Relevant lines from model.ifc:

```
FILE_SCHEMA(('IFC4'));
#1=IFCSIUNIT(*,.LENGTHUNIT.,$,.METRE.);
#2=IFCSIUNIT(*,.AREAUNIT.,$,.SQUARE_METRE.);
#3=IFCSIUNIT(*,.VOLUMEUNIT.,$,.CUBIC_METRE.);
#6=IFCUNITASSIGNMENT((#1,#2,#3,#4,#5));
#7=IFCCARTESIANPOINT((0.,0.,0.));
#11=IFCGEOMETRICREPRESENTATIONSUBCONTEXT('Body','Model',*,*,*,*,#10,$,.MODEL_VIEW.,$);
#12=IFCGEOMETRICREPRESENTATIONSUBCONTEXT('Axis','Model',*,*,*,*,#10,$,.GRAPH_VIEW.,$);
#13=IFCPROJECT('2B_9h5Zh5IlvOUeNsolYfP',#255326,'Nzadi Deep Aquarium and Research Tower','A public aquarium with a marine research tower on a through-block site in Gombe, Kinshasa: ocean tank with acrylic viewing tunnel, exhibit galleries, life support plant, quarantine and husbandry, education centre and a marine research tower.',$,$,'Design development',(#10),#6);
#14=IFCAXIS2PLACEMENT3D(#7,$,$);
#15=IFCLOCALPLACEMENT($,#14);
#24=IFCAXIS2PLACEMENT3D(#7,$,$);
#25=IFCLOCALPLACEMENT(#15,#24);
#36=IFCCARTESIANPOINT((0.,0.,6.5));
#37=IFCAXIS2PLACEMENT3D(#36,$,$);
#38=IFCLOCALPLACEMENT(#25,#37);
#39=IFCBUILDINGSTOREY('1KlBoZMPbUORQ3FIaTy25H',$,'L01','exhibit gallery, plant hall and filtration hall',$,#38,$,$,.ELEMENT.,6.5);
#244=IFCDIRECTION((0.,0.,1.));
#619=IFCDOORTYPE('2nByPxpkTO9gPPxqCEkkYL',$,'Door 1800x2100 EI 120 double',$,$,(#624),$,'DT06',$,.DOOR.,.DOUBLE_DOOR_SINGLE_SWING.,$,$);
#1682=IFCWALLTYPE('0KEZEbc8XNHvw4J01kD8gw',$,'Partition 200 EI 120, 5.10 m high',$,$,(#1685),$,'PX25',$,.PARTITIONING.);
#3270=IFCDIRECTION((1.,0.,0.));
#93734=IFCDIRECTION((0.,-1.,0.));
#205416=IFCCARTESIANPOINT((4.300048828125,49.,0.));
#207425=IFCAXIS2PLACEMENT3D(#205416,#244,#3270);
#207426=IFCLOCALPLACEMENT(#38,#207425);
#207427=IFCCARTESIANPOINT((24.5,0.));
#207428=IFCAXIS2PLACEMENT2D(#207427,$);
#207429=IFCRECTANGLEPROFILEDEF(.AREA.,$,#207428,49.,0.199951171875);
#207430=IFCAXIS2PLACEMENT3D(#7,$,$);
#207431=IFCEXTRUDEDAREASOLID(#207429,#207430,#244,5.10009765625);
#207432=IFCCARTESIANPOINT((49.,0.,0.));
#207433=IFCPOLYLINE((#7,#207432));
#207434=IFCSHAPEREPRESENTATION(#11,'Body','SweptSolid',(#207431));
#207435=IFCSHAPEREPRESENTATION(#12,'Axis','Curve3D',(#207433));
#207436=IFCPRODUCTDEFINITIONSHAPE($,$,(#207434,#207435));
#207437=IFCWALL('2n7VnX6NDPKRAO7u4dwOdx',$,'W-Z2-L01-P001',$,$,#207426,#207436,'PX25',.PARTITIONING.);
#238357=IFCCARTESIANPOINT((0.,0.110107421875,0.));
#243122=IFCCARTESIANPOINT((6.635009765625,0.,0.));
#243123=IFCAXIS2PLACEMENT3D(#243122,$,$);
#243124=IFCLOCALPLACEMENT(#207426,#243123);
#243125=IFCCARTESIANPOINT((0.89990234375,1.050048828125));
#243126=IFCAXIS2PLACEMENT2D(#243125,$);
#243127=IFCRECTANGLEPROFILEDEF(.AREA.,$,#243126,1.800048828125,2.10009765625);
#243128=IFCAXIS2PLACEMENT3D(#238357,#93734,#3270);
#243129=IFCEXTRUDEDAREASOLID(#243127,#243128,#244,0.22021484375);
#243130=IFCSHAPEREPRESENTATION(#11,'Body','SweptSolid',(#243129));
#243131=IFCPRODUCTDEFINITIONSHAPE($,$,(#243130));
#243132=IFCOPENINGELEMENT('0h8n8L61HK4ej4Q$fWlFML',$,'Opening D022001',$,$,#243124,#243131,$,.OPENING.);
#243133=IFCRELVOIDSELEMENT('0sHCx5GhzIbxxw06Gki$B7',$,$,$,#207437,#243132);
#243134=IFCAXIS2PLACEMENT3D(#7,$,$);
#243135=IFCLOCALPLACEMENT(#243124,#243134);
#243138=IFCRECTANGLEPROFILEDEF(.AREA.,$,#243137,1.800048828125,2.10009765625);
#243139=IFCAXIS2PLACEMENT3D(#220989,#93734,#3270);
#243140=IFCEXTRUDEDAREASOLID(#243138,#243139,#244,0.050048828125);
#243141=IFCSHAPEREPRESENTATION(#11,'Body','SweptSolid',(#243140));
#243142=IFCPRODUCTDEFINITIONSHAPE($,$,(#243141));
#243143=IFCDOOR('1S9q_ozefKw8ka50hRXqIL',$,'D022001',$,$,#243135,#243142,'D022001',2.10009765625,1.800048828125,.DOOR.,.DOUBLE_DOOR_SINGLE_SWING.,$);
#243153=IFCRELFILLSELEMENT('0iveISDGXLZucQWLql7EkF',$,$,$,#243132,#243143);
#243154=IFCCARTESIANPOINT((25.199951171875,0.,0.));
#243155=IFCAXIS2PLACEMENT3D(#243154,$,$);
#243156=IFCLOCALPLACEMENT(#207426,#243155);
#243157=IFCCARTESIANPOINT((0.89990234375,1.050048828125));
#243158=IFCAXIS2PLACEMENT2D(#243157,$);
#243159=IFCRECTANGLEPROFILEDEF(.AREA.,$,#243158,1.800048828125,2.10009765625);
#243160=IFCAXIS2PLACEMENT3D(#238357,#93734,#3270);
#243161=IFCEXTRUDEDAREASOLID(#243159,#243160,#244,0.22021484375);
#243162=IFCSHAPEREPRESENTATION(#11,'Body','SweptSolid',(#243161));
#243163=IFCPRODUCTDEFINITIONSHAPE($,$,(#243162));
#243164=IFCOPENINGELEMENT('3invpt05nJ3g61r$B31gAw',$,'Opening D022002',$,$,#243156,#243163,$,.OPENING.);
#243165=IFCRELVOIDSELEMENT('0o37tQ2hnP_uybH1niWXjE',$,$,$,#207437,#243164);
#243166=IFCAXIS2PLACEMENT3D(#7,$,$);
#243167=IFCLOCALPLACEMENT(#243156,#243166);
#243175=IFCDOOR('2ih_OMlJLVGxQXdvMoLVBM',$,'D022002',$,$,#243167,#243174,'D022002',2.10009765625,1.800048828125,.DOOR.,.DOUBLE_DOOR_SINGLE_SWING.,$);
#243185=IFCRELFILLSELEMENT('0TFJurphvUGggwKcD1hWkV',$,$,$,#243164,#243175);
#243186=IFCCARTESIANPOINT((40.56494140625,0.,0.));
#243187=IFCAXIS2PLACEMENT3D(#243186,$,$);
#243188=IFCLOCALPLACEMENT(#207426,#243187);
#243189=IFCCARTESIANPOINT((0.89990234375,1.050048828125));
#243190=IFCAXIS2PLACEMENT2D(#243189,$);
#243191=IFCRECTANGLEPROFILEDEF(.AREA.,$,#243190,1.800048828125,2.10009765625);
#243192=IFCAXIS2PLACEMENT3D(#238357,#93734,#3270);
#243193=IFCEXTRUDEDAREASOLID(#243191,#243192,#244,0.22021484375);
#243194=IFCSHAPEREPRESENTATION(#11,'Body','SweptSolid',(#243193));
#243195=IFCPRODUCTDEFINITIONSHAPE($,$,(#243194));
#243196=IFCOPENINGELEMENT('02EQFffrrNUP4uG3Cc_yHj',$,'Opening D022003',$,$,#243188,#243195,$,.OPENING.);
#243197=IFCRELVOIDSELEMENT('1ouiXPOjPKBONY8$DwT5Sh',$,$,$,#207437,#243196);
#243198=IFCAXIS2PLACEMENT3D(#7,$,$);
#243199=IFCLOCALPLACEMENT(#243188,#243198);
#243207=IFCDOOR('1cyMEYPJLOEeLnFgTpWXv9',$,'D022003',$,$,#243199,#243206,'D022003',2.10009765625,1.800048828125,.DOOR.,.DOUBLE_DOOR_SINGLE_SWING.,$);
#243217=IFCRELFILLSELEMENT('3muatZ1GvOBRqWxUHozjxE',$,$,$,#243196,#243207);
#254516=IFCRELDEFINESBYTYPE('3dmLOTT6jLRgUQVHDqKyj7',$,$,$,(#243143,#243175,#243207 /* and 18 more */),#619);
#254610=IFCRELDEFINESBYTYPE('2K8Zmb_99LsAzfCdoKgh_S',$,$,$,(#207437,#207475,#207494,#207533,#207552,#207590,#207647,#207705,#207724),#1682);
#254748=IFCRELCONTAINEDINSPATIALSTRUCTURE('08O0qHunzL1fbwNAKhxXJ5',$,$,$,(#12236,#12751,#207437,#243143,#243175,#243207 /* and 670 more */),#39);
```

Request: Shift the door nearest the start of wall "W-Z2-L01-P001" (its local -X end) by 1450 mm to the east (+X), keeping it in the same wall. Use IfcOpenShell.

```python
import ifcopenshell
import ifcopenshell.api.geometry
import ifcopenshell.util.placement

model = ifcopenshell.open("model.ifc")

door = model.by_guid("1S9q_ozefKw8ka50hRXqIL")
opening = door.FillsVoids[0].RelatingOpeningElement
wall = opening.VoidsElements[0].RelatingBuildingElement

wall_matrix = ifcopenshell.util.placement.get_local_placement(wall.ObjectPlacement)
shift = wall_matrix[:3, 0] * 1.45
before = ifcopenshell.util.placement.get_local_placement(door.ObjectPlacement)[:3, 3].copy()

# The door is placed relative to its opening, so it follows when the opening moves.
matrix = ifcopenshell.util.placement.get_local_placement(opening.ObjectPlacement)
matrix[:3, 3] += shift
ifcopenshell.api.geometry.edit_object_placement(
    model, product=opening, matrix=matrix, is_si=False, should_transform_children=True
)

after = ifcopenshell.util.placement.get_local_placement(door.ObjectPlacement)[:3, 3]
print("door moved by", (after - before).round(3) + 0.0)

model.write("model_edited.ifc")
```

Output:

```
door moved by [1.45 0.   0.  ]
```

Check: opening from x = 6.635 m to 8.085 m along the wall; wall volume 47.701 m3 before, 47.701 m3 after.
